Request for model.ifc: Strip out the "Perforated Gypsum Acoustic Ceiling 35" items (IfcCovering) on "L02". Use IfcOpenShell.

First a look at what the model holds.

```python
import ifcopenshell
import ifcopenshell.util.element

model = ifcopenshell.open("model.ifc")
print(model.schema)
storey = next(s for s in model.by_type("IfcBuildingStorey") if s.Name == "L02")
coverings = [e for e in ifcopenshell.util.element.get_decomposition(storey) if e.is_a("IfcCovering")]
seen = {}
for e in coverings:
    element_type = ifcopenshell.util.element.get_type(e)
    name = element_type.Name if element_type not in (None, e) else None
    seen[name] = seen.get(name, 0) + 1
for name, count in sorted(seen.items(), key=str):
    print(count, "x", name)
```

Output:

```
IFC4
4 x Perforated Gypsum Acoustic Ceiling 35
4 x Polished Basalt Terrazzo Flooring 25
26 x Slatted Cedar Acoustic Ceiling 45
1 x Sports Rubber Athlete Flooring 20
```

```python
import ifcopenshell
import ifcopenshell.api.root
import ifcopenshell.util.element

model = ifcopenshell.open("model.ifc")

storey = next(s for s in model.by_type("IfcBuildingStorey") if s.Name == "L02")
coverings = [e for e in ifcopenshell.util.element.get_decomposition(storey) if e.is_a("IfcCovering")]
targets = [e for e in coverings if (t := ifcopenshell.util.element.get_type(e)) not in (None, e) and t.Name == "Perforated Gypsum Acoustic Ceiling 35"]

for e in targets:
    ifcopenshell.api.root.remove_product(model, product=e)
print(len(targets), "removed")

model.write("model_updated.ifc")
```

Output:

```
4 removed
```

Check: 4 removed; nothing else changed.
